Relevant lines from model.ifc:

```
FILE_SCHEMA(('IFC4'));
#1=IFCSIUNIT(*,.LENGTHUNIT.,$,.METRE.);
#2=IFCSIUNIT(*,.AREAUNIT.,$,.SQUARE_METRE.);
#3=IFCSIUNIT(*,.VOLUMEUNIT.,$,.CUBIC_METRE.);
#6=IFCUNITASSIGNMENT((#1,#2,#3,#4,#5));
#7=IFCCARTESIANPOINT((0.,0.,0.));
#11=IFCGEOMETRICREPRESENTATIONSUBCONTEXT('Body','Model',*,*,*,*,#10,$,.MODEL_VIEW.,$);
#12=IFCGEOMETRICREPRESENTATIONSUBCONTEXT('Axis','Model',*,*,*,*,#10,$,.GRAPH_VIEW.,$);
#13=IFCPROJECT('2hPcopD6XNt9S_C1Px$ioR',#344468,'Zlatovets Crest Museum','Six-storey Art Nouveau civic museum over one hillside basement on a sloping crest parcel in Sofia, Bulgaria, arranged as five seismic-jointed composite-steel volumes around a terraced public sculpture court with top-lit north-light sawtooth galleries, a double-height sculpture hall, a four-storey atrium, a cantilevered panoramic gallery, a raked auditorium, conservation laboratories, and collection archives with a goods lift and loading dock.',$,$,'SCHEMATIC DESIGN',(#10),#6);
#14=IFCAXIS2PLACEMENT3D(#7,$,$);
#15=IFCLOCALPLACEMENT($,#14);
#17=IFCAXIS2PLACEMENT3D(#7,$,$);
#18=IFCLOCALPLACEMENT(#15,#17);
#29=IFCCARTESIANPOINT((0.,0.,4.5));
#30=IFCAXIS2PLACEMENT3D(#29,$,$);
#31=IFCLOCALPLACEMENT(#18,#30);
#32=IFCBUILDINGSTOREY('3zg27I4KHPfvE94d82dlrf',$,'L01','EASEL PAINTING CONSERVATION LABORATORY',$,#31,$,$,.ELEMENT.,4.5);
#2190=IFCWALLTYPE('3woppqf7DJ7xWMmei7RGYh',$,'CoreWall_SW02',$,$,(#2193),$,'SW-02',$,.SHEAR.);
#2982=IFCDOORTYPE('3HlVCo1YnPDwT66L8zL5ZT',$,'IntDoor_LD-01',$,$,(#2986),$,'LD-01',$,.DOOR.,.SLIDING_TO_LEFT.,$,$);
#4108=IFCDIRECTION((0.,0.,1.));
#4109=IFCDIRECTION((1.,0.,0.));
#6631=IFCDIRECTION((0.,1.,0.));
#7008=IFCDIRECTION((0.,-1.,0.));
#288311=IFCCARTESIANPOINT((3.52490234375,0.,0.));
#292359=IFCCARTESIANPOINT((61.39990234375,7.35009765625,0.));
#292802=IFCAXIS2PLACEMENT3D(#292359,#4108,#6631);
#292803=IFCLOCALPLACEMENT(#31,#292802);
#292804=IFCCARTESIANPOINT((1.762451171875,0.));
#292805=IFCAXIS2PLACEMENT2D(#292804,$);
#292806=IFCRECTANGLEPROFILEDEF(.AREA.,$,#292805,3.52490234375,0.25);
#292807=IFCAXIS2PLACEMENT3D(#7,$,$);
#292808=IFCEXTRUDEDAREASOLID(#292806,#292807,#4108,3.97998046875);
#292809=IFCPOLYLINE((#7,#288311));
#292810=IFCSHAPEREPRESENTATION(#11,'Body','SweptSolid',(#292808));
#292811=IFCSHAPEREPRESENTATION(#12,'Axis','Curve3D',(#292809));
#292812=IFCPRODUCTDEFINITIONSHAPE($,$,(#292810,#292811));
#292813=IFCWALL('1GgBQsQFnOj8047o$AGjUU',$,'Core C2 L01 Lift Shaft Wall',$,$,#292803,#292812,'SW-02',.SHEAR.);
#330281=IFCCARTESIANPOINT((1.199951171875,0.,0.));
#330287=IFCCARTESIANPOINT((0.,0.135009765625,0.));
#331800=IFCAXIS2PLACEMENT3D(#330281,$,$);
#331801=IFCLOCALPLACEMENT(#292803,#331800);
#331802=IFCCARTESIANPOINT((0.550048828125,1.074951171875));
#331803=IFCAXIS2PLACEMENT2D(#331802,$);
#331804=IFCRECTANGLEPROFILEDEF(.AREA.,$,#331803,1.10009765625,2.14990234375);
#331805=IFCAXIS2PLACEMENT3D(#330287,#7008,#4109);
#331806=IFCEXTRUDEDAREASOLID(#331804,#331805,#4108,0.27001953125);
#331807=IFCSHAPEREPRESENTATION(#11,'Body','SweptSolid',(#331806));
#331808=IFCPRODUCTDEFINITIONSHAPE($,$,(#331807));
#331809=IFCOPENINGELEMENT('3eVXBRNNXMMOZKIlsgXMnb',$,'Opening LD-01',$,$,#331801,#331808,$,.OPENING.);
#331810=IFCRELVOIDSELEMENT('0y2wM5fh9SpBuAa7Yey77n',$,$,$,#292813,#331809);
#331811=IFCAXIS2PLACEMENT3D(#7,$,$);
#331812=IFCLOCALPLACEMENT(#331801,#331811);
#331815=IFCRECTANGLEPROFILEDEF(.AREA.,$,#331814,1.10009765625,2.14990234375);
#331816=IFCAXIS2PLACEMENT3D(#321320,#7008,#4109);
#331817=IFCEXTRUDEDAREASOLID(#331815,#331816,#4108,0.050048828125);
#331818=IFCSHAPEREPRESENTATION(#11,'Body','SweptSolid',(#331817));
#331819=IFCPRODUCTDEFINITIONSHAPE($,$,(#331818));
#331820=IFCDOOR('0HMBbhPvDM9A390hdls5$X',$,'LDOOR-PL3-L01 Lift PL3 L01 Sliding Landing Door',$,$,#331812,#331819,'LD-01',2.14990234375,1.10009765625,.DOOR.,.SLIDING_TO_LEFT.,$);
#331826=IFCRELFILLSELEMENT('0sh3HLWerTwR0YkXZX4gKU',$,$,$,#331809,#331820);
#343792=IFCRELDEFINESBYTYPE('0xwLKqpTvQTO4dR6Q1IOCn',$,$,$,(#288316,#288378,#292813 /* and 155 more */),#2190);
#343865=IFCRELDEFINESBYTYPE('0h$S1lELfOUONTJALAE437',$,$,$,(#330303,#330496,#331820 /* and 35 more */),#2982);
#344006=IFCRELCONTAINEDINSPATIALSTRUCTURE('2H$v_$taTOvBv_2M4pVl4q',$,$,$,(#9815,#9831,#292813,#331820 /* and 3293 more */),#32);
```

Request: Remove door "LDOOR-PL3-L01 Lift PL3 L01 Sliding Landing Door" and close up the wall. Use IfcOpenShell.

```python
import ifcopenshell
import ifcopenshell.api.feature
import ifcopenshell.api.root
import ifcopenshell.geom
import ifcopenshell.util.shape

model = ifcopenshell.open("model.ifc")
settings = ifcopenshell.geom.settings()


def volume(element):
    """Net volume in cubic metres, openings subtracted."""
    shape = ifcopenshell.geom.create_shape(settings, element)
    return ifcopenshell.util.shape.get_volume(shape.geometry)


door = model.by_guid("0HMBbhPvDM9A390hdls5$X")
opening = door.FillsVoids[0].RelatingOpeningElement
wall = opening.VoidsElements[0].RelatingBuildingElement
before = volume(wall)

ifcopenshell.api.root.remove_product(model, product=door)
ifcopenshell.api.feature.remove_feature(model, feature=opening)

after = volume(wall)

print(f"wall volume {before:.3f} -> {after:.3f} m3")

model.write("model-out.ifc")
```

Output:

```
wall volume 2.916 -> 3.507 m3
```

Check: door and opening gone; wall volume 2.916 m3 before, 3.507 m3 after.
